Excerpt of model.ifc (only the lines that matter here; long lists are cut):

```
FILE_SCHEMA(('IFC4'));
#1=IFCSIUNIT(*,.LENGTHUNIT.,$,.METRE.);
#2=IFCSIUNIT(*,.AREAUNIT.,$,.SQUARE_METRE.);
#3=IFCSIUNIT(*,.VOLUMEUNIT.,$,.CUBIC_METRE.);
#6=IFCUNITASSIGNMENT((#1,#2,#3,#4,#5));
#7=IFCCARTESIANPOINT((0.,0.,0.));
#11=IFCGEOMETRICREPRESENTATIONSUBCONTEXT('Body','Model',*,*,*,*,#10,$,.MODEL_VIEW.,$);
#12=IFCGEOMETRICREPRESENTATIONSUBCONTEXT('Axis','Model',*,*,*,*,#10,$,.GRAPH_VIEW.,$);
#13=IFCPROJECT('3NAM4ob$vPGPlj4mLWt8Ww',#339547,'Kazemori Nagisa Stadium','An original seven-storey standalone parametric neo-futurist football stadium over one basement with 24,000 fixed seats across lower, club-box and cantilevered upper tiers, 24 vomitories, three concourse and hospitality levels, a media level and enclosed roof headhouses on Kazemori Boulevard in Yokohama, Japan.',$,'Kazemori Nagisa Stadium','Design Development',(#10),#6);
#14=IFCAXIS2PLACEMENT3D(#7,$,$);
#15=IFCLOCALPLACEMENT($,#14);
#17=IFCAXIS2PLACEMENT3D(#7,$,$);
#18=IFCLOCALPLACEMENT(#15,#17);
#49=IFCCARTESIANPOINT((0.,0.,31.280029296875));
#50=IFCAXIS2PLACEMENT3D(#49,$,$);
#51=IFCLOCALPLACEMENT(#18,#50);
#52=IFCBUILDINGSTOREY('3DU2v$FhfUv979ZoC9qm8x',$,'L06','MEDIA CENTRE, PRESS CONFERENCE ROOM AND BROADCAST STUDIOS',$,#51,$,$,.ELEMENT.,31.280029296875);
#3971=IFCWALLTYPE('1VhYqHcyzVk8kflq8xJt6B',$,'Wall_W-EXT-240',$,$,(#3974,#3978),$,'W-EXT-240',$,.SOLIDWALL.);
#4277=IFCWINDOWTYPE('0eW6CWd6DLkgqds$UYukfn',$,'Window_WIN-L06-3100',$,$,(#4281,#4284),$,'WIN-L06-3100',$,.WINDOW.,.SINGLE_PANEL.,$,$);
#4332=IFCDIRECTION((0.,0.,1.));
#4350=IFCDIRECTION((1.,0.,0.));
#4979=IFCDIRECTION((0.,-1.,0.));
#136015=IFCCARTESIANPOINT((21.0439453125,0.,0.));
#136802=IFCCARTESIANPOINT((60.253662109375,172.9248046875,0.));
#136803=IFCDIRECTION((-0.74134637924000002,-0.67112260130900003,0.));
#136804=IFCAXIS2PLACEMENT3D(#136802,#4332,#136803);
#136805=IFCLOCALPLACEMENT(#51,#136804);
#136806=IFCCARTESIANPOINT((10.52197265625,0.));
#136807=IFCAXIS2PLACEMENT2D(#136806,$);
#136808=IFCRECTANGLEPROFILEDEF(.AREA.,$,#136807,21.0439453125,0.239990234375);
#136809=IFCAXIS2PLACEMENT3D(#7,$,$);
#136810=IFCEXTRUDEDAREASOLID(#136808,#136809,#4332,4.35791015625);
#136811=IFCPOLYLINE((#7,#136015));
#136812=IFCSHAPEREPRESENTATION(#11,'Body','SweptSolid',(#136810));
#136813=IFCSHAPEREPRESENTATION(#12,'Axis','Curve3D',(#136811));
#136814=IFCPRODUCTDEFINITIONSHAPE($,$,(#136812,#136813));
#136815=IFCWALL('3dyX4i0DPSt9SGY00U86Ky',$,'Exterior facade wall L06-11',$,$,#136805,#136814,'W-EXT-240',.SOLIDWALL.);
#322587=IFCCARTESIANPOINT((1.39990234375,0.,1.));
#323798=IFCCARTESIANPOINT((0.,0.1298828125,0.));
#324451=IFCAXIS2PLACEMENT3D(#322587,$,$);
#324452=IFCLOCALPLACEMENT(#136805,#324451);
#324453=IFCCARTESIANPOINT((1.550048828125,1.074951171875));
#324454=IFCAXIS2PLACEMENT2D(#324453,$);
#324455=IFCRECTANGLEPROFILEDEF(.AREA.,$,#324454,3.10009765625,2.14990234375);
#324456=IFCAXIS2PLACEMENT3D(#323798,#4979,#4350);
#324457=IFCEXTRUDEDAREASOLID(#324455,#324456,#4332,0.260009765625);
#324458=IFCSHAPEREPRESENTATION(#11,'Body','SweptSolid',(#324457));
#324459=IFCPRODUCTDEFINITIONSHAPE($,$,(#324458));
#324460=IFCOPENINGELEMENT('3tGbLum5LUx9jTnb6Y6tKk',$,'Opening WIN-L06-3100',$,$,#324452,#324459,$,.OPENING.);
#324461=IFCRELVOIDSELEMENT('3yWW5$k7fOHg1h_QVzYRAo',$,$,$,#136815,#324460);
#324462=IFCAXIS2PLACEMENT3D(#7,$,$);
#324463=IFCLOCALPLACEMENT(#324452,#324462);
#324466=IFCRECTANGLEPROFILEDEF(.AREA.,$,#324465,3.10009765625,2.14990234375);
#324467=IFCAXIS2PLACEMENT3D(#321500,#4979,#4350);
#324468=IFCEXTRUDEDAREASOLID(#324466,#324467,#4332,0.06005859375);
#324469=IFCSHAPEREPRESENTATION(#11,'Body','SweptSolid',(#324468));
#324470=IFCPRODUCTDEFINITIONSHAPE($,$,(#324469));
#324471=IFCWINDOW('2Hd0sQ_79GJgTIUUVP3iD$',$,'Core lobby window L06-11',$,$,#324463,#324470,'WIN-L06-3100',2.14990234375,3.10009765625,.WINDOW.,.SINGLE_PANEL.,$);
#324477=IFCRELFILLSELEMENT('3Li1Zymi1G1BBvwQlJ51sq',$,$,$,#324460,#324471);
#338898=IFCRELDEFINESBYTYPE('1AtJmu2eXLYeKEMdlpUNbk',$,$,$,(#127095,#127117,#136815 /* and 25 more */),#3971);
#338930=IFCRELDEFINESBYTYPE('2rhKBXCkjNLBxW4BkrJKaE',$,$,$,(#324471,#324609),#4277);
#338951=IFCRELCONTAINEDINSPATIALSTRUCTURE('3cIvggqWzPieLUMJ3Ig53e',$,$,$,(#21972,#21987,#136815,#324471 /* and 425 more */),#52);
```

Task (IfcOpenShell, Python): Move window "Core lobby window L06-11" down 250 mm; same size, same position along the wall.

```python
import numpy as np
import ifcopenshell
import ifcopenshell.api.geometry
import ifcopenshell.util.placement
import ifcopenshell.util.unit

model = ifcopenshell.open("model.ifc")
unit_scale = ifcopenshell.util.unit.calculate_unit_scale(model)

window = model.by_guid("2Hd0sQ_79GJgTIUUVP3iD$")
opening = window.FillsVoids[0].RelatingOpeningElement
dz = -0.25 / unit_scale

shift = np.array([0.0, 0.0, dz])
# The window is placed relative to its opening, so it follows when the opening moves.
matrix = ifcopenshell.util.placement.get_local_placement(opening.ObjectPlacement)
matrix[:3, 3] += shift
ifcopenshell.api.geometry.edit_object_placement(
    model, product=opening, matrix=matrix, is_si=False, should_transform_children=True
)

print(f"moved by {dz * unit_scale:+.3f} m")

model.write("model_edited.ifc")
```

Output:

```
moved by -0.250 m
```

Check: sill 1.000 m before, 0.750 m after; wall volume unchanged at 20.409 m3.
